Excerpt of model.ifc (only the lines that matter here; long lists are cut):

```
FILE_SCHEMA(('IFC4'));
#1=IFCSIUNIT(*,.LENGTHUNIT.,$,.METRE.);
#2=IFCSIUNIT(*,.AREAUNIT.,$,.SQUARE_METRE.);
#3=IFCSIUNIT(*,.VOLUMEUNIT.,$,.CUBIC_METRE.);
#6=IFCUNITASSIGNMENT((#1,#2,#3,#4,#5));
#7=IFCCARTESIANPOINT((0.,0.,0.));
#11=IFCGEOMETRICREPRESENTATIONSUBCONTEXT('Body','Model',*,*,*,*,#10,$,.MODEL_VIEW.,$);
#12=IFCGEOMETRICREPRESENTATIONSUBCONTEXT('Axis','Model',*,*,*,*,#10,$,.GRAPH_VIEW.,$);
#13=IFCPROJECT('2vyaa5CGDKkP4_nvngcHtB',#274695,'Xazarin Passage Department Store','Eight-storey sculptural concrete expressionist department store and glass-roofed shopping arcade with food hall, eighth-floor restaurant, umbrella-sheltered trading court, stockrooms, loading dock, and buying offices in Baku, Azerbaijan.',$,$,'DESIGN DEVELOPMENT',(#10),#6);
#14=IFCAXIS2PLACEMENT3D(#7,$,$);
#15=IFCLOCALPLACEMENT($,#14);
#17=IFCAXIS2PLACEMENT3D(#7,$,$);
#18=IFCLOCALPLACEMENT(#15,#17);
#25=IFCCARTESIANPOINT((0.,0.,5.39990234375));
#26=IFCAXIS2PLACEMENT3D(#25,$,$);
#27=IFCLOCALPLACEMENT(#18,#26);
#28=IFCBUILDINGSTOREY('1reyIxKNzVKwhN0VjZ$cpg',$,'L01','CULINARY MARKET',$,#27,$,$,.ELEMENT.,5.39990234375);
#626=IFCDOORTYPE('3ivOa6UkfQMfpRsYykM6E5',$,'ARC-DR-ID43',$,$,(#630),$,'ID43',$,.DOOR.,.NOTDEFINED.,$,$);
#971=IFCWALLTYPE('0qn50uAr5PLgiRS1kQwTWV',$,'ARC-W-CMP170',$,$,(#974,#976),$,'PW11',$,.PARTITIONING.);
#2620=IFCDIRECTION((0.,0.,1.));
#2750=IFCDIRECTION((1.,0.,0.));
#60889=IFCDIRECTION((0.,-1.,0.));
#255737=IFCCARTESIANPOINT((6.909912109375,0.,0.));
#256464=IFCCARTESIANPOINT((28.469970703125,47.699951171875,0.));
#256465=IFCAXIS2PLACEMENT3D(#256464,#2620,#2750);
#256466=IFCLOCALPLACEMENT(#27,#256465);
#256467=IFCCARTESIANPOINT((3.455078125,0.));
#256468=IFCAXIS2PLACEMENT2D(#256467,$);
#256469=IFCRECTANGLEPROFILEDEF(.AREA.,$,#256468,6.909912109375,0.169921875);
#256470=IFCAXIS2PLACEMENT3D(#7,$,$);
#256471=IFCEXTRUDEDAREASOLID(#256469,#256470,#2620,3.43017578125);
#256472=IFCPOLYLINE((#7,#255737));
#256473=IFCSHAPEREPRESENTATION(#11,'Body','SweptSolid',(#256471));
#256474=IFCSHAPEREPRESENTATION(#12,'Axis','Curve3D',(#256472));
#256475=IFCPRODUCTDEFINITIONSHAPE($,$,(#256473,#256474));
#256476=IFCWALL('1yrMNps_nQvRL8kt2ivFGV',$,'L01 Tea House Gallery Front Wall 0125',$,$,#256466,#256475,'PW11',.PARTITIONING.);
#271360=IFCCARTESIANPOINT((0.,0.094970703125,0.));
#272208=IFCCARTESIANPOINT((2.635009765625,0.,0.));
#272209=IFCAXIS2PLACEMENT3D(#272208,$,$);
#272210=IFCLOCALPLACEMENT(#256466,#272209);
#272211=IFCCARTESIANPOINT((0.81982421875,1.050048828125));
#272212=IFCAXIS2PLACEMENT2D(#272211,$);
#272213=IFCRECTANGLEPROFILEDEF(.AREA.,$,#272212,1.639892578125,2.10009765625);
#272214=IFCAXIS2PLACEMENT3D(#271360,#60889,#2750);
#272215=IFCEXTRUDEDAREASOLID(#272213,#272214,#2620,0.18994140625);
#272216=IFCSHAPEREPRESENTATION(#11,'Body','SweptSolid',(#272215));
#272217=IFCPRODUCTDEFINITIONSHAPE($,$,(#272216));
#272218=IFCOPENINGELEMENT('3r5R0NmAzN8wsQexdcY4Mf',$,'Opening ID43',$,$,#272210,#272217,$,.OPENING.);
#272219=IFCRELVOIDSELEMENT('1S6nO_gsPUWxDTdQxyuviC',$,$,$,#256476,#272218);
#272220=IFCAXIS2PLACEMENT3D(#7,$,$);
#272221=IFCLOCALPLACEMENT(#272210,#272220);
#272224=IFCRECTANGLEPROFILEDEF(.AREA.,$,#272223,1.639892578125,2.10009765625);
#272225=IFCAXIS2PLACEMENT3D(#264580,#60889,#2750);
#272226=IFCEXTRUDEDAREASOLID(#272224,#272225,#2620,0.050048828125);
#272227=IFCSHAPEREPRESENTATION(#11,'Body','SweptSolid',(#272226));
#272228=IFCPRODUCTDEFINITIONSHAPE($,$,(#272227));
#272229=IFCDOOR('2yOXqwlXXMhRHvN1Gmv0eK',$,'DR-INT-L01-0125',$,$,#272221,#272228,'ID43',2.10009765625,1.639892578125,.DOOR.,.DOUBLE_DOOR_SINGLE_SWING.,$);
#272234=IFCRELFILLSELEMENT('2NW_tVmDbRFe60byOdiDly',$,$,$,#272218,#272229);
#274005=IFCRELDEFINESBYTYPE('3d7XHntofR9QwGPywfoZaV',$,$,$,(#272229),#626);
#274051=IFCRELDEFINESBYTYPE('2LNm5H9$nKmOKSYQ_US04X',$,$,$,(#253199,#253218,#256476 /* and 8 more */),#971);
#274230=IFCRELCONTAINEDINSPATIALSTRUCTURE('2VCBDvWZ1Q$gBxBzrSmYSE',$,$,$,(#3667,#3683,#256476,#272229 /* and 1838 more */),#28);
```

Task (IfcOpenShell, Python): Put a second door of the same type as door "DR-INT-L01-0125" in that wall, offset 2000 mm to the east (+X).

```python
import ifcopenshell
import ifcopenshell.api.feature
import ifcopenshell.api.geometry
import ifcopenshell.api.root
import ifcopenshell.geom
import ifcopenshell.util.element
import ifcopenshell.util.placement
import ifcopenshell.util.shape
import ifcopenshell.util.unit

model = ifcopenshell.open("model.ifc")
unit_scale = ifcopenshell.util.unit.calculate_unit_scale(model)
settings = ifcopenshell.geom.settings()


def volume(element):
    """Net volume in cubic metres, openings subtracted."""
    shape = ifcopenshell.geom.create_shape(settings, element)
    return ifcopenshell.util.shape.get_volume(shape.geometry)


door = model.by_guid("2yOXqwlXXMhRHvN1Gmv0eK")
opening = door.FillsVoids[0].RelatingOpeningElement
wall = opening.VoidsElements[0].RelatingBuildingElement
before = volume(wall)
shift = ifcopenshell.util.placement.get_local_placement(wall.ObjectPlacement)[:3, 0] * 2 / unit_scale

# copy_class copies the void relationship, type, container and properties, but no geometry.
new_opening = ifcopenshell.api.root.copy_class(model, product=opening)
new_opening.Representation = ifcopenshell.util.element.copy_deep(
    model, opening.Representation, exclude=["IfcGeometricRepresentationContext", "IfcRepresentationMap"]
)
new_door = ifcopenshell.api.root.copy_class(model, product=door)
new_door.Representation = ifcopenshell.util.element.copy_deep(
    model, door.Representation, exclude=["IfcGeometricRepresentationContext", "IfcRepresentationMap"]
)
new_door.Tag = None
ifcopenshell.api.feature.add_filling(model, opening=new_opening, element=new_door)

for old, new in ((opening, new_opening), (door, new_door)):
    matrix = ifcopenshell.util.placement.get_local_placement(old.ObjectPlacement)
    matrix[:3, 3] += shift
    ifcopenshell.api.geometry.edit_object_placement(model, product=new, matrix=matrix, is_si=False)

after = volume(wall)

print(f"wall volume {before:.3f} -> {after:.3f} m3")

model.write("model_updated.ifc")
```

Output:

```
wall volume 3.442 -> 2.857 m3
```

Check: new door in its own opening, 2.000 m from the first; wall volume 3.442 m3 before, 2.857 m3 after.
